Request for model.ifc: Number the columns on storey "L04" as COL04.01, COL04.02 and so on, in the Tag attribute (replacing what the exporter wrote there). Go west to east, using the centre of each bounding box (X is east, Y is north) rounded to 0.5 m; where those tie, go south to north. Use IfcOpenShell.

First a look at what the model holds.

```python
import ifcopenshell
import ifcopenshell.util.element
import ifcopenshell.util.placement

model = ifcopenshell.open("model.ifc")
print(model.schema)
storey = next(s for s in model.by_type("IfcBuildingStorey") if s.Name == "L04")
columns = [e for e in ifcopenshell.util.element.get_decomposition(storey) if e.is_a("IfcColumn")]
for e in sorted(columns, key=lambda e: e.id()):
    origin = ifcopenshell.util.placement.get_local_placement(e.ObjectPlacement)[:3, 3]
    print(e.id(), e.Tag, e.Name, origin.round(2) + 0.0, sep=" | ")
```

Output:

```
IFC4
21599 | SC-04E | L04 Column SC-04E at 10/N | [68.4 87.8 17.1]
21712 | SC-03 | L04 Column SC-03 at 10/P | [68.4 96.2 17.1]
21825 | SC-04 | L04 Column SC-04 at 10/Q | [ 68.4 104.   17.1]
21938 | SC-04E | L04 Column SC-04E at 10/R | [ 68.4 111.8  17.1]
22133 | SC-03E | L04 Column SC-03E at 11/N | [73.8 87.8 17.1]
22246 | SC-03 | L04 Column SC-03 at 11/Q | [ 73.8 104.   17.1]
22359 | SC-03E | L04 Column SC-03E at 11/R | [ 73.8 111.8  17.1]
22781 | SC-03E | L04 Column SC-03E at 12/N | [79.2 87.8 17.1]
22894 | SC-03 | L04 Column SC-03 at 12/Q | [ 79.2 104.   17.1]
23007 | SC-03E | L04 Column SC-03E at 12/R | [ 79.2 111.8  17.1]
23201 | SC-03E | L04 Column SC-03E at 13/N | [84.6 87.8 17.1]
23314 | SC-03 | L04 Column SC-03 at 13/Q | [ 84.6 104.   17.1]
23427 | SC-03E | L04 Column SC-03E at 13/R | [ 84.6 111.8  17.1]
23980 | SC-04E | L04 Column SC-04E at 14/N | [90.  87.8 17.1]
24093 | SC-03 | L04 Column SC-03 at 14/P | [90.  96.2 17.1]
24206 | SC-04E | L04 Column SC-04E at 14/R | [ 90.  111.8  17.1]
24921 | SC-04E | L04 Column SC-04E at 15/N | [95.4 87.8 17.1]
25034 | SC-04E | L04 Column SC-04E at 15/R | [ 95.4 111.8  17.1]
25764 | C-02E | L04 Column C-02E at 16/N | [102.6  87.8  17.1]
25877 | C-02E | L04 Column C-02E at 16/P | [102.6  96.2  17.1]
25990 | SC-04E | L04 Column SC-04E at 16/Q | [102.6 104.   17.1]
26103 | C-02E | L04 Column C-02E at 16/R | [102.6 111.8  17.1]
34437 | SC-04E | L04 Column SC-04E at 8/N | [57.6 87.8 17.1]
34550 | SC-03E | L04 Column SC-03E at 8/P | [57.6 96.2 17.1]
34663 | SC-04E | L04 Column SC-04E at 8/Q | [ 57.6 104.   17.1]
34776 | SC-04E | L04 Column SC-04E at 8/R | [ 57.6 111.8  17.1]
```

```python
import ifcopenshell
import ifcopenshell.geom
import ifcopenshell.util.element
import ifcopenshell.util.shape

model = ifcopenshell.open("model.ifc")
settings = ifcopenshell.geom.settings()
settings.set("use-world-coords", True)


def centre(element):
    shape = ifcopenshell.geom.create_shape(settings, element)
    return ifcopenshell.util.shape.get_bbox_centroid(shape.geometry)


storey = next(s for s in model.by_type("IfcBuildingStorey") if s.Name == "L04")
columns = [e for e in ifcopenshell.util.element.get_decomposition(storey) if e.is_a("IfcColumn")]

# Insertion points can sit at a corner or the storey origin, so sort by the geometry (in metres).
centres = {e: centre(e) for e in columns}
columns.sort(key=lambda e: (round(centres[e][0] / 0.5), centres[e][1]))

for i, e in enumerate(columns, start=1):
    number = f"COL04.{i:02d}"
    e.Tag = number
    print(e.id(), number)

model.write("model-out.ifc")
```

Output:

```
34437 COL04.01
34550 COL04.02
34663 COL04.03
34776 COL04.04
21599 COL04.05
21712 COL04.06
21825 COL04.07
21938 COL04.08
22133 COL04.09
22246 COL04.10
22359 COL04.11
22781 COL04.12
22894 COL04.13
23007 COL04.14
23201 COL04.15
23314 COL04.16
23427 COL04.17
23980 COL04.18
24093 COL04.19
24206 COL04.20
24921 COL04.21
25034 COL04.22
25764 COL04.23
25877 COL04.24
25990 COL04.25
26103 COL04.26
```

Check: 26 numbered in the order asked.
